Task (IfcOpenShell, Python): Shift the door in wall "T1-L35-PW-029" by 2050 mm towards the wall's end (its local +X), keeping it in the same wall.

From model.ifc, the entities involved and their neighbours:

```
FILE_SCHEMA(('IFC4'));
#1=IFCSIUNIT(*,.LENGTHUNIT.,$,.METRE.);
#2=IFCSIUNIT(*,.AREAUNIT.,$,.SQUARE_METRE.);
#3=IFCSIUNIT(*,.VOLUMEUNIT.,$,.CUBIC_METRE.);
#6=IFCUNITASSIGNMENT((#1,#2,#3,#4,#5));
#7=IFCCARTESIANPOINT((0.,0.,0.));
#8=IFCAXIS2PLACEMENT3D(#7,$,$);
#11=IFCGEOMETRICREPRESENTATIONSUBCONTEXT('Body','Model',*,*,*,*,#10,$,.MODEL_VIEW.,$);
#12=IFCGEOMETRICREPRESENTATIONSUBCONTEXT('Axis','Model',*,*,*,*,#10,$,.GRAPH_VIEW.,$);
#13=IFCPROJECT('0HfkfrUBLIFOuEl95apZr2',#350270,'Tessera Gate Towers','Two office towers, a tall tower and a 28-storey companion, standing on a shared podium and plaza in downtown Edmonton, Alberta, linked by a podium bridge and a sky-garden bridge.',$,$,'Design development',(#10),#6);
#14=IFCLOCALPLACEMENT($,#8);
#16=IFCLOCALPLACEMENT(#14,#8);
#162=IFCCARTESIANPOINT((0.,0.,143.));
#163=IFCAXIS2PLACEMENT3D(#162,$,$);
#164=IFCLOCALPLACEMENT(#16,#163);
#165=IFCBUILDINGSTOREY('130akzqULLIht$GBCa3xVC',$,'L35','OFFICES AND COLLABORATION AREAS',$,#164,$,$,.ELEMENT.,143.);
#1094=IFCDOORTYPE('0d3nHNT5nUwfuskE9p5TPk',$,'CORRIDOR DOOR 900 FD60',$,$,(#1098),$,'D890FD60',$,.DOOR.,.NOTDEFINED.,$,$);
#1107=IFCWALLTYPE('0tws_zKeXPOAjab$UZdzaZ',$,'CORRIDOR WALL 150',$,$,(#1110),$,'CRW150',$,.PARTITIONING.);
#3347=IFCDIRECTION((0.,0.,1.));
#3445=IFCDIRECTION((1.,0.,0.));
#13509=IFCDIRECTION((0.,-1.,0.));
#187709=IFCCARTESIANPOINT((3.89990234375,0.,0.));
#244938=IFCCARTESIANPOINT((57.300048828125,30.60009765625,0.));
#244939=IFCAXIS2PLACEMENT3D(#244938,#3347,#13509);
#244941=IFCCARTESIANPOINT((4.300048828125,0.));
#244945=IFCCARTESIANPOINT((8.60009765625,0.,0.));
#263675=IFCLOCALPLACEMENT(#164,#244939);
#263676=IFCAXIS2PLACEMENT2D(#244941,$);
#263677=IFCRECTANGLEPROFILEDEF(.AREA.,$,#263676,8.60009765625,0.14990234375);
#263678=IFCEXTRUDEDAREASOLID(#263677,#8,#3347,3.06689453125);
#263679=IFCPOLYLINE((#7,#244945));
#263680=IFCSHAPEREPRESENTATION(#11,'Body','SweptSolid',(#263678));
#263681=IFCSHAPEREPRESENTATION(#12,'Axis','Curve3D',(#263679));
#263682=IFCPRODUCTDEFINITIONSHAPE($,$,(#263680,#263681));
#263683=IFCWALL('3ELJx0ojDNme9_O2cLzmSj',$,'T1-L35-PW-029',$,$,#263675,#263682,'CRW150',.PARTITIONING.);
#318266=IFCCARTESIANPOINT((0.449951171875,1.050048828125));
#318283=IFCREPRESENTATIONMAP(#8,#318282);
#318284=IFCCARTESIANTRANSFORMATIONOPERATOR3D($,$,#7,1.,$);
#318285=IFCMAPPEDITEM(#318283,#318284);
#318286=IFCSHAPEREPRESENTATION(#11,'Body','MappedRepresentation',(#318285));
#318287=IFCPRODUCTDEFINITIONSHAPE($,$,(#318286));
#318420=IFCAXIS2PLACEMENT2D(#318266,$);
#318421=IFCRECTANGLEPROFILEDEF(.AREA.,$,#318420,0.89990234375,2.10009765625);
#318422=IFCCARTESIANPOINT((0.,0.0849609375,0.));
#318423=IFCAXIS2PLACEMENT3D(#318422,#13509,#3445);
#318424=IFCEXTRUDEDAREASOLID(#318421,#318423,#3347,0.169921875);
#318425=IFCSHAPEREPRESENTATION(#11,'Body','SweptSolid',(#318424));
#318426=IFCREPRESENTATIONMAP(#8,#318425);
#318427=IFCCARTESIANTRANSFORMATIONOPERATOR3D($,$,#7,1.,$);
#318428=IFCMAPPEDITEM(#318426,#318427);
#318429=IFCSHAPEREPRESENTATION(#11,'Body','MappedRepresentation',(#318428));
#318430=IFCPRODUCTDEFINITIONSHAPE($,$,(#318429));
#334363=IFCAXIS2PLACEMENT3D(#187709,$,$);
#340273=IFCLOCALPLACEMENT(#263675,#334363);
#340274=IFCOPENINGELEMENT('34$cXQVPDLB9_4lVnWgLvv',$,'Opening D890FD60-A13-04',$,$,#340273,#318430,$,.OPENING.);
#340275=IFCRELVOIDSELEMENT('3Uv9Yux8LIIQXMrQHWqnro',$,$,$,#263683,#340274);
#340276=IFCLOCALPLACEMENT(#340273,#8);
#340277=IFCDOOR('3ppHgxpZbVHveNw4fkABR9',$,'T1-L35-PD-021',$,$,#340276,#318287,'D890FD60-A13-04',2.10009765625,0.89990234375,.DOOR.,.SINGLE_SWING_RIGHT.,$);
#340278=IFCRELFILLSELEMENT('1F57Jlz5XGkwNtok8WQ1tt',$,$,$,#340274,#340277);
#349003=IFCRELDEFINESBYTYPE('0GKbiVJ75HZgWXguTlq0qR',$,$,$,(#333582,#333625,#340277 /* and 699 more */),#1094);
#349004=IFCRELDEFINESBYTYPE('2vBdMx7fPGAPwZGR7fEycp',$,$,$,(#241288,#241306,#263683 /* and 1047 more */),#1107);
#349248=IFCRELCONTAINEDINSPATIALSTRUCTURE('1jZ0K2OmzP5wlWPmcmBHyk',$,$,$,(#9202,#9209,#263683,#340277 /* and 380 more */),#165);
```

```python
import ifcopenshell
import ifcopenshell.api.geometry
import ifcopenshell.util.placement
import ifcopenshell.util.unit

model = ifcopenshell.open("model.ifc")
unit_scale = ifcopenshell.util.unit.calculate_unit_scale(model)

door = model.by_guid("3ppHgxpZbVHveNw4fkABR9")
opening = door.FillsVoids[0].RelatingOpeningElement
wall = opening.VoidsElements[0].RelatingBuildingElement

wall_matrix = ifcopenshell.util.placement.get_local_placement(wall.ObjectPlacement)
shift = wall_matrix[:3, 0] * 2.05 / unit_scale
before = ifcopenshell.util.placement.get_local_placement(door.ObjectPlacement)[:3, 3].copy()

# The door is placed relative to its opening, so it follows when the opening moves.
matrix = ifcopenshell.util.placement.get_local_placement(opening.ObjectPlacement)
matrix[:3, 3] += shift
ifcopenshell.api.geometry.edit_object_placement(
    model, product=opening, matrix=matrix, is_si=False, should_transform_children=True
)

after = ifcopenshell.util.placement.get_local_placement(door.ObjectPlacement)[:3, 3]
print("door moved by", (after - before).round(3) + 0.0)

model.write("model_rev.ifc")
```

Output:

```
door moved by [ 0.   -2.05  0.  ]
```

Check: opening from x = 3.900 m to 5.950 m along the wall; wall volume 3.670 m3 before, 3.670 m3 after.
